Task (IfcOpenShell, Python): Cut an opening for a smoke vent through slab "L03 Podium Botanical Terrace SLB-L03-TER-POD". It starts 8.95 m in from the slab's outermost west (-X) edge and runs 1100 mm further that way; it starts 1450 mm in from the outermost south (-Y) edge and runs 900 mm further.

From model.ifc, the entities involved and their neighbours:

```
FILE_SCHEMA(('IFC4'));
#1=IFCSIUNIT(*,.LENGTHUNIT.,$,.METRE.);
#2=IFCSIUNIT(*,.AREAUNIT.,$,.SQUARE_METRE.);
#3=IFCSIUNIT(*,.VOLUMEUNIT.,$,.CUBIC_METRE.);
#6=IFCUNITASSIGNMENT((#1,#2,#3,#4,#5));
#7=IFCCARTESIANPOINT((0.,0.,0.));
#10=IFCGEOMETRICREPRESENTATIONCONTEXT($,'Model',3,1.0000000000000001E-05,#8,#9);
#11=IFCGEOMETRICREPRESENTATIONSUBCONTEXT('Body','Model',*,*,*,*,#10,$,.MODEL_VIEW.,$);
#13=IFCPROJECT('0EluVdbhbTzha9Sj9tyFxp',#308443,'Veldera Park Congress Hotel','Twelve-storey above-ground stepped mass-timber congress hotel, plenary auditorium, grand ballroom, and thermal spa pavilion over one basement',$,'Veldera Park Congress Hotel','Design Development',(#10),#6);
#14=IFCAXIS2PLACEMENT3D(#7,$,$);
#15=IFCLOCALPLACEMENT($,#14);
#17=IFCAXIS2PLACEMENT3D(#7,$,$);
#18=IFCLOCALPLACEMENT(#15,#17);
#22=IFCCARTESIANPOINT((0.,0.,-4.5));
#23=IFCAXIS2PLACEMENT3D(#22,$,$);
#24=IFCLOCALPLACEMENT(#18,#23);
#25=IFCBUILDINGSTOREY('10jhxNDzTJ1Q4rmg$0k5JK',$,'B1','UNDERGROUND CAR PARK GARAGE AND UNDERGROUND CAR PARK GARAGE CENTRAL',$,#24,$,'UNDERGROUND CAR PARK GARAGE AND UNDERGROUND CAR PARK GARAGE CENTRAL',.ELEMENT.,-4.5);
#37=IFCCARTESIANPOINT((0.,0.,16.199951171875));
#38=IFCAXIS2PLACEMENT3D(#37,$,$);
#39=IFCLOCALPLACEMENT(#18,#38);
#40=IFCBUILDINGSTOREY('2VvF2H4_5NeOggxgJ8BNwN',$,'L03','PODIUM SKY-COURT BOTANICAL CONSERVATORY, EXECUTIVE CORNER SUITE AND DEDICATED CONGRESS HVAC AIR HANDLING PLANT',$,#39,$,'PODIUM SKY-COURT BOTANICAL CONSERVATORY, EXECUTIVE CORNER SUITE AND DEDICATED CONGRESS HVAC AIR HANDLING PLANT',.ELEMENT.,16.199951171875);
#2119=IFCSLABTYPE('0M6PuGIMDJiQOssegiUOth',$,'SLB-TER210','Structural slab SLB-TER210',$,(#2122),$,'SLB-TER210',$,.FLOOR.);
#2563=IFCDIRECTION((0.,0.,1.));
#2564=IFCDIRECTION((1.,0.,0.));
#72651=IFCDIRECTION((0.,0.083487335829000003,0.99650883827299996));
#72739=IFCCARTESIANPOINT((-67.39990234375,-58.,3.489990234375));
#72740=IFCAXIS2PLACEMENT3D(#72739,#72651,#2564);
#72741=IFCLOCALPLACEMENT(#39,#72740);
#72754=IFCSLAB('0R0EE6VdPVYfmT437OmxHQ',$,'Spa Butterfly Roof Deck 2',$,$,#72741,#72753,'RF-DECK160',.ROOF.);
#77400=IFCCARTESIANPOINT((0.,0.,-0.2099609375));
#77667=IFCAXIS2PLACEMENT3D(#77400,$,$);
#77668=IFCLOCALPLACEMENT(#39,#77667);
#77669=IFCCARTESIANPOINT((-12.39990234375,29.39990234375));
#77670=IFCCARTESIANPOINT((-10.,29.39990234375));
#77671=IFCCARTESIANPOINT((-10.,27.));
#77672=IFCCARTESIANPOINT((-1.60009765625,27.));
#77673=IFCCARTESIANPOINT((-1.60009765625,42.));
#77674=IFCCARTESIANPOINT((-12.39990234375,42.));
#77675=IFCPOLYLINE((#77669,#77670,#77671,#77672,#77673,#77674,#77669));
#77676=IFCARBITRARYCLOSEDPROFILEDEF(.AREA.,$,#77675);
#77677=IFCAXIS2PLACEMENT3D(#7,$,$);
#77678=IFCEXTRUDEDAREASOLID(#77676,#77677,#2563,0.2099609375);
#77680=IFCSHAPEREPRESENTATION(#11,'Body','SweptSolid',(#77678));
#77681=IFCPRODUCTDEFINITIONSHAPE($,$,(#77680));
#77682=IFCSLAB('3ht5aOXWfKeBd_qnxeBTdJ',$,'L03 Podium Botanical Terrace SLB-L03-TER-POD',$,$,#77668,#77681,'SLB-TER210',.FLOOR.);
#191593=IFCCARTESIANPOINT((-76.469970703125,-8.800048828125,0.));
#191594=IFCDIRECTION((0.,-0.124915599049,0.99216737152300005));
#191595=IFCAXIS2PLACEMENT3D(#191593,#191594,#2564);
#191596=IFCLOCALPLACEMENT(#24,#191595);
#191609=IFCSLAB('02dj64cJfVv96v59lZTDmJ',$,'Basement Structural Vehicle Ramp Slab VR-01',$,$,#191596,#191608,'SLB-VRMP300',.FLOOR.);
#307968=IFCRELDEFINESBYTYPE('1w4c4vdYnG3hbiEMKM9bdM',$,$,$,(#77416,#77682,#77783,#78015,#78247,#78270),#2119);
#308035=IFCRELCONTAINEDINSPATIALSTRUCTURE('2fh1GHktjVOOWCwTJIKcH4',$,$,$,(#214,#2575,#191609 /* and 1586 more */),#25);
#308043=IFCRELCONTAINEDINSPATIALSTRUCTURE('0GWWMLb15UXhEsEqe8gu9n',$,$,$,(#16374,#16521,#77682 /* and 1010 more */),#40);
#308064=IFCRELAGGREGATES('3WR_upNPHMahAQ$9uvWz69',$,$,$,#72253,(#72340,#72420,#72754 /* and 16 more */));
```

```python
import numpy as np
import ifcopenshell
import ifcopenshell.api.feature
import ifcopenshell.api.geometry
import ifcopenshell.api.root
import ifcopenshell.geom
import ifcopenshell.util.placement
import ifcopenshell.util.representation
import ifcopenshell.util.shape
import ifcopenshell.util.unit

model = ifcopenshell.open("model.ifc")
unit_scale = ifcopenshell.util.unit.calculate_unit_scale(model)
settings = ifcopenshell.geom.settings()


def volume(element):
    """Net volume in cubic metres, openings subtracted."""
    shape = ifcopenshell.geom.create_shape(settings, element)
    return ifcopenshell.util.shape.get_volume(shape.geometry)


slab = model.by_guid("3ht5aOXWfKeBd_qnxeBTdJ")
before = volume(slab)

# Extent in the slab's own axes, in metres. The edges named are its -X and -Y sides.
slab_shape = ifcopenshell.geom.create_shape(settings, slab)
vertices = ifcopenshell.util.shape.get_vertices(slab_shape.geometry)
x_min, y_min, bottom = vertices.min(axis=0)
top = vertices[:, 2].max()

opening = ifcopenshell.api.root.create_entity(model, ifc_class="IfcOpeningElement", name="Smoke vent opening", predefined_type="OPENING")
context = ifcopenshell.util.representation.get_context(model, "Model", "Body", "MODEL_VIEW")
width, depth = 1.1, 0.9
outline = [(0.0, 0.0), (width, 0.0), (width, depth), (0.0, depth), (0.0, 0.0)]
# Overshoot both faces by 50 mm so the cut is clean.
shape = ifcopenshell.api.geometry.add_slab_representation(
    model, context=context, depth=top - bottom + 0.1, polyline=outline
)
ifcopenshell.api.geometry.assign_representation(model, product=opening, representation=shape)

matrix = ifcopenshell.util.placement.get_local_placement(slab.ObjectPlacement)
matrix[:, 3] = matrix @ np.append(np.array([x_min + 8.95, y_min + 1.45, bottom - 0.05]) / unit_scale, 1.0)
ifcopenshell.api.geometry.edit_object_placement(model, product=opening, matrix=matrix, is_si=False)
ifcopenshell.api.feature.add_feature(model, feature=opening, element=slab)

after = volume(slab)

print(f"slab volume {before:.3f} -> {after:.3f} m3")

model.write("model_updated.ifc")
```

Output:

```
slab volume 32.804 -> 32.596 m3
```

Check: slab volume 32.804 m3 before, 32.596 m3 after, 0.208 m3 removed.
